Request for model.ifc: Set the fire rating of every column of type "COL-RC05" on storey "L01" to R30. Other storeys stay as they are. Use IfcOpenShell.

First a look at what the model holds.

```python
import ifcopenshell
import ifcopenshell.util.element

model = ifcopenshell.open("model.ifc")
print(model.schema)
storey = next(s for s in model.by_type("IfcBuildingStorey") if s.Name == "L01")
columns = [e for e in ifcopenshell.util.element.get_decomposition(storey) if e.is_a("IfcColumn")]
seen = {}
for e in columns:
    element_type = ifcopenshell.util.element.get_type(e)
    key = (element_type.Name if element_type != e and element_type else None, ifcopenshell.util.element.get_pset(e, "Pset_ColumnCommon", "FireRating"))
    seen[key] = seen.get(key, 0) + 1
for (name, value), count in sorted(seen.items(), key=str):
    print(count, "x", name, "|", value)
```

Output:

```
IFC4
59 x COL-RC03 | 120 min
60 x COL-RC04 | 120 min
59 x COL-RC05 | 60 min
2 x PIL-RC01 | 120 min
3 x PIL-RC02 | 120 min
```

```python
import ifcopenshell
import ifcopenshell.api.pset
import ifcopenshell.util.element

model = ifcopenshell.open("model.ifc")

storey = next(s for s in model.by_type("IfcBuildingStorey") if s.Name == "L01")
columns = [e for e in ifcopenshell.util.element.get_decomposition(storey) if e.is_a("IfcColumn")]

count = 0
for e in columns:
    element_type = ifcopenshell.util.element.get_type(e)
    if element_type in (None, e) or element_type.Name != "COL-RC05":
        continue
    # add_pset returns the element's existing set when there is one.
    pset = ifcopenshell.api.pset.add_pset(model, product=e, name="Pset_ColumnCommon")
    ifcopenshell.api.pset.edit_pset(model, pset=pset, properties={"FireRating": "R30"})
    count += 1

print(count, "columns updated")

model.write("model_edited.ifc")
```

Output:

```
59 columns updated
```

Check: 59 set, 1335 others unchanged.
